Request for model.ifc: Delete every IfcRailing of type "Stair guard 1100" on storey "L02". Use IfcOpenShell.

First a look at what the model holds.

```python
import ifcopenshell
import ifcopenshell.util.element

model = ifcopenshell.open("model.ifc")
print(model.schema)
storey = next(s for s in model.by_type("IfcBuildingStorey") if s.Name == "L02")
railings = [e for e in ifcopenshell.util.element.get_decomposition(storey) if e.is_a("IfcRailing")]
seen = {}
for e in railings:
    element_type = ifcopenshell.util.element.get_type(e)
    name = element_type.Name if element_type not in (None, e) else None
    seen[name] = seen.get(name, 0) + 1
for name, count in sorted(seen.items(), key=str):
    print(count, "x", name)
```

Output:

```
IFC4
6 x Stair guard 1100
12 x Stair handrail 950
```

```python
import ifcopenshell
import ifcopenshell.api.root
import ifcopenshell.util.element

model = ifcopenshell.open("model.ifc")

storey = next(s for s in model.by_type("IfcBuildingStorey") if s.Name == "L02")
railings = [e for e in ifcopenshell.util.element.get_decomposition(storey) if e.is_a("IfcRailing")]
targets = [e for e in railings if (t := ifcopenshell.util.element.get_type(e)) not in (None, e) and t.Name == "Stair guard 1100"]

for e in targets:
    ifcopenshell.api.root.remove_product(model, product=e)
print(len(targets), "removed")

model.write("model_edited.ifc")
```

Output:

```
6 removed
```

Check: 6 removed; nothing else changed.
